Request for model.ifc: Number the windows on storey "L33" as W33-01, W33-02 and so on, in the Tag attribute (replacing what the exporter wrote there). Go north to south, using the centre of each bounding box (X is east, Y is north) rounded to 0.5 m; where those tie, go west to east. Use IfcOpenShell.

First a look at what the model holds.

```python
import ifcopenshell
import ifcopenshell.util.element
import ifcopenshell.util.placement

model = ifcopenshell.open("model.ifc")
print(model.schema)
storey = next(s for s in model.by_type("IfcBuildingStorey") if s.Name == "L33")
windows = [e for e in ifcopenshell.util.element.get_decomposition(storey) if e.is_a("IfcWindow")]
for e in sorted(windows, key=lambda e: e.id()):
    origin = ifcopenshell.util.placement.get_local_placement(e.ObjectPlacement)[:3, 3]
    print(e.id(), e.Tag, e.Name, origin.round(2) + 0.0, sep=" | ")
```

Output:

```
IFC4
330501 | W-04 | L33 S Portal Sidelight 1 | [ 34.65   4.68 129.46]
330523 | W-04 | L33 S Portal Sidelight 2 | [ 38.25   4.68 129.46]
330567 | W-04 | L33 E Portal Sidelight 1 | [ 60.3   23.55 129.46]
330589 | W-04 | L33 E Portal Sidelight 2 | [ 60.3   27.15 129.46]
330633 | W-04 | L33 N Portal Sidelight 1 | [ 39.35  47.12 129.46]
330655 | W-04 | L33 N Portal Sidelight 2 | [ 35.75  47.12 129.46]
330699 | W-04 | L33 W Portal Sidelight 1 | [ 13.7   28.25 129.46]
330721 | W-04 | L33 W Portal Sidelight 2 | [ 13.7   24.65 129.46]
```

```python
import ifcopenshell
import ifcopenshell.geom
import ifcopenshell.util.element
import ifcopenshell.util.shape

model = ifcopenshell.open("model.ifc")
settings = ifcopenshell.geom.settings()
settings.set("use-world-coords", True)


def centre(element):
    shape = ifcopenshell.geom.create_shape(settings, element)
    return ifcopenshell.util.shape.get_bbox_centroid(shape.geometry)


storey = next(s for s in model.by_type("IfcBuildingStorey") if s.Name == "L33")
windows = [e for e in ifcopenshell.util.element.get_decomposition(storey) if e.is_a("IfcWindow")]

# Insertion points can sit at a corner or the storey origin, so sort by the geometry (in metres).
centres = {e: centre(e) for e in windows}
windows.sort(key=lambda e: (-round(centres[e][1] / 0.5), centres[e][0]))

for i, e in enumerate(windows, start=1):
    number = f"W33-{i:02d}"
    e.Tag = number
    print(e.id(), number)

model.write("model_updated.ifc")
```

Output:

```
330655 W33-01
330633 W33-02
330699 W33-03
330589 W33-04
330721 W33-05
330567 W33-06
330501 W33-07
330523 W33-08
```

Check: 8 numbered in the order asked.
